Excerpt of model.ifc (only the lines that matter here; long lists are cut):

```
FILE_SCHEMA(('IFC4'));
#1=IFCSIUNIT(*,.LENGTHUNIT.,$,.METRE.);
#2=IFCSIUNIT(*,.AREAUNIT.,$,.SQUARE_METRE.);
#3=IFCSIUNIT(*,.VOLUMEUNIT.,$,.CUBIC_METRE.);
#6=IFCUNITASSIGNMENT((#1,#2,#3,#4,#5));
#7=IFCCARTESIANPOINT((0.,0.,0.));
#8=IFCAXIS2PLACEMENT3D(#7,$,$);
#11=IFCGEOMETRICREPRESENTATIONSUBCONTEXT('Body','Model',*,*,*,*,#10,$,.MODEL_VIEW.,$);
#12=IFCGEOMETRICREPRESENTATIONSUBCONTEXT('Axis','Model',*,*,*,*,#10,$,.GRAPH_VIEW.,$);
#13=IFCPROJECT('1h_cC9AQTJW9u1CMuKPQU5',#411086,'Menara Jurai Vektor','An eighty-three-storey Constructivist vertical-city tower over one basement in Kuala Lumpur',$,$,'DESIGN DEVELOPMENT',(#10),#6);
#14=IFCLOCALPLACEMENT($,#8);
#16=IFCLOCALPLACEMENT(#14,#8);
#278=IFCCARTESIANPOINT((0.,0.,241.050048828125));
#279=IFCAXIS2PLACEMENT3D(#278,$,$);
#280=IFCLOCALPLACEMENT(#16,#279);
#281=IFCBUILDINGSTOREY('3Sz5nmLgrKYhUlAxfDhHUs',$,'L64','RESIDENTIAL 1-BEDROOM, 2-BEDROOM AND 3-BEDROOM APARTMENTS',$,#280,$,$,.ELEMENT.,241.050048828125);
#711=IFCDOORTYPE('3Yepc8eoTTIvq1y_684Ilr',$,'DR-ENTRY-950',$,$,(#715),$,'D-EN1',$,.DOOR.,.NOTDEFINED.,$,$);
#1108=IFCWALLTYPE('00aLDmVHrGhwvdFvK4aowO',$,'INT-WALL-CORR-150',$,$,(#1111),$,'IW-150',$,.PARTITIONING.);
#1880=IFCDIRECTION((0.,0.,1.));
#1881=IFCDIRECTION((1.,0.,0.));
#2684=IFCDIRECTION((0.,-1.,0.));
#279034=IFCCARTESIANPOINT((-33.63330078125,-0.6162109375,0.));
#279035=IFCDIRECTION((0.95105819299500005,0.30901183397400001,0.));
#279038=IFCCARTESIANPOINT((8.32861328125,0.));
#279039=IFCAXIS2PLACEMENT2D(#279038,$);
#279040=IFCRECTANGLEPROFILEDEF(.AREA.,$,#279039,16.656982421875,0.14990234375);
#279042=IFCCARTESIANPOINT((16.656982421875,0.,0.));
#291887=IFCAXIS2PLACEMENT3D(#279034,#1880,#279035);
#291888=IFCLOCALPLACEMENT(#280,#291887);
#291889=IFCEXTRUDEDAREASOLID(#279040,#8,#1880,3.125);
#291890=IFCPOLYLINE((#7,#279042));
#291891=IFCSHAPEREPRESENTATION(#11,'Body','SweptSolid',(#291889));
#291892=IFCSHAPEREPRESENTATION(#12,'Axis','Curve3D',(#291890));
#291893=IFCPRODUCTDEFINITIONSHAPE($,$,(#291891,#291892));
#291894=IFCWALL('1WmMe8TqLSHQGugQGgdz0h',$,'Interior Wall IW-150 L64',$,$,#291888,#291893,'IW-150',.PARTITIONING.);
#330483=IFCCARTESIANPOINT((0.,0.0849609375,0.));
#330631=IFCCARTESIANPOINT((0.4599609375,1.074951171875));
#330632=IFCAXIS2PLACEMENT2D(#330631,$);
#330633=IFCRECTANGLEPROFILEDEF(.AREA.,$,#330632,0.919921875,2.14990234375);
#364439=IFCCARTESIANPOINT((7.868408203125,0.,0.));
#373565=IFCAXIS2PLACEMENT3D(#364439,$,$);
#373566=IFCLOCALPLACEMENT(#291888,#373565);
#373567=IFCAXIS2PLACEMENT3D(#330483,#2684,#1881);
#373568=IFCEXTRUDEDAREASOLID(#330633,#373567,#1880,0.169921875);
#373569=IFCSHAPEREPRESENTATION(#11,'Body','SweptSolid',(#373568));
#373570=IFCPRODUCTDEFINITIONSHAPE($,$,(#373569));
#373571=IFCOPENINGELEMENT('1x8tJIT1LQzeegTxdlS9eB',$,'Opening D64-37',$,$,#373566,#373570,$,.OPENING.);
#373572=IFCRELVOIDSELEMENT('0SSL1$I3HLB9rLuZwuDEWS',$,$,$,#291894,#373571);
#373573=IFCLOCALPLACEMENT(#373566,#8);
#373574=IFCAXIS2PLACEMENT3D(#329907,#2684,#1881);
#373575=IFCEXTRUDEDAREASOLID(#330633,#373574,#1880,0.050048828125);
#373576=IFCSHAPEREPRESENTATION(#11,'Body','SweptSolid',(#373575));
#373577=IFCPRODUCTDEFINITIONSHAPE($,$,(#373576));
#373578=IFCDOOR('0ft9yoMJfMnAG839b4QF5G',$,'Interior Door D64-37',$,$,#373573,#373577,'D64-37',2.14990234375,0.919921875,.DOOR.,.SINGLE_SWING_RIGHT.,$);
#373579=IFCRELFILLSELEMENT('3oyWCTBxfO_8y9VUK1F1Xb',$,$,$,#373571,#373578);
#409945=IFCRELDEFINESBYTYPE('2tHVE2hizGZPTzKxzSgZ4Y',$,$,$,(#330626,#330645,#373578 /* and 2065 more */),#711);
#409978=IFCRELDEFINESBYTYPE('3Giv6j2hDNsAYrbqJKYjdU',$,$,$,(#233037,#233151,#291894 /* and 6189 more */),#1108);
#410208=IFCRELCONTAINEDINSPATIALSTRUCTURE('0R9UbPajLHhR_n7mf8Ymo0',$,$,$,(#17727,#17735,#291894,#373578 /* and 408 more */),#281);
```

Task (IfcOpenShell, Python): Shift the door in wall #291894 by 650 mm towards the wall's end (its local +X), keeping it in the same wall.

```python
import ifcopenshell
import ifcopenshell.api.geometry
import ifcopenshell.util.placement
import ifcopenshell.util.unit

model = ifcopenshell.open("model.ifc")
unit_scale = ifcopenshell.util.unit.calculate_unit_scale(model)

door = model.by_guid("0ft9yoMJfMnAG839b4QF5G")
opening = door.FillsVoids[0].RelatingOpeningElement
wall = opening.VoidsElements[0].RelatingBuildingElement

wall_matrix = ifcopenshell.util.placement.get_local_placement(wall.ObjectPlacement)
shift = wall_matrix[:3, 0] * 0.65 / unit_scale
before = ifcopenshell.util.placement.get_local_placement(door.ObjectPlacement)[:3, 3].copy()

# The door is placed relative to its opening, so it follows when the opening moves.
matrix = ifcopenshell.util.placement.get_local_placement(opening.ObjectPlacement)
matrix[:3, 3] += shift
ifcopenshell.api.geometry.edit_object_placement(
    model, product=opening, matrix=matrix, is_si=False, should_transform_children=True
)

after = ifcopenshell.util.placement.get_local_placement(door.ObjectPlacement)[:3, 3]
print("door moved by", (after - before).round(3) + 0.0)

model.write("model_v2.ifc")
```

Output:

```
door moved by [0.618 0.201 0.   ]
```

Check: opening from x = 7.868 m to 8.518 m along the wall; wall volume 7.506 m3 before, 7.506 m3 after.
